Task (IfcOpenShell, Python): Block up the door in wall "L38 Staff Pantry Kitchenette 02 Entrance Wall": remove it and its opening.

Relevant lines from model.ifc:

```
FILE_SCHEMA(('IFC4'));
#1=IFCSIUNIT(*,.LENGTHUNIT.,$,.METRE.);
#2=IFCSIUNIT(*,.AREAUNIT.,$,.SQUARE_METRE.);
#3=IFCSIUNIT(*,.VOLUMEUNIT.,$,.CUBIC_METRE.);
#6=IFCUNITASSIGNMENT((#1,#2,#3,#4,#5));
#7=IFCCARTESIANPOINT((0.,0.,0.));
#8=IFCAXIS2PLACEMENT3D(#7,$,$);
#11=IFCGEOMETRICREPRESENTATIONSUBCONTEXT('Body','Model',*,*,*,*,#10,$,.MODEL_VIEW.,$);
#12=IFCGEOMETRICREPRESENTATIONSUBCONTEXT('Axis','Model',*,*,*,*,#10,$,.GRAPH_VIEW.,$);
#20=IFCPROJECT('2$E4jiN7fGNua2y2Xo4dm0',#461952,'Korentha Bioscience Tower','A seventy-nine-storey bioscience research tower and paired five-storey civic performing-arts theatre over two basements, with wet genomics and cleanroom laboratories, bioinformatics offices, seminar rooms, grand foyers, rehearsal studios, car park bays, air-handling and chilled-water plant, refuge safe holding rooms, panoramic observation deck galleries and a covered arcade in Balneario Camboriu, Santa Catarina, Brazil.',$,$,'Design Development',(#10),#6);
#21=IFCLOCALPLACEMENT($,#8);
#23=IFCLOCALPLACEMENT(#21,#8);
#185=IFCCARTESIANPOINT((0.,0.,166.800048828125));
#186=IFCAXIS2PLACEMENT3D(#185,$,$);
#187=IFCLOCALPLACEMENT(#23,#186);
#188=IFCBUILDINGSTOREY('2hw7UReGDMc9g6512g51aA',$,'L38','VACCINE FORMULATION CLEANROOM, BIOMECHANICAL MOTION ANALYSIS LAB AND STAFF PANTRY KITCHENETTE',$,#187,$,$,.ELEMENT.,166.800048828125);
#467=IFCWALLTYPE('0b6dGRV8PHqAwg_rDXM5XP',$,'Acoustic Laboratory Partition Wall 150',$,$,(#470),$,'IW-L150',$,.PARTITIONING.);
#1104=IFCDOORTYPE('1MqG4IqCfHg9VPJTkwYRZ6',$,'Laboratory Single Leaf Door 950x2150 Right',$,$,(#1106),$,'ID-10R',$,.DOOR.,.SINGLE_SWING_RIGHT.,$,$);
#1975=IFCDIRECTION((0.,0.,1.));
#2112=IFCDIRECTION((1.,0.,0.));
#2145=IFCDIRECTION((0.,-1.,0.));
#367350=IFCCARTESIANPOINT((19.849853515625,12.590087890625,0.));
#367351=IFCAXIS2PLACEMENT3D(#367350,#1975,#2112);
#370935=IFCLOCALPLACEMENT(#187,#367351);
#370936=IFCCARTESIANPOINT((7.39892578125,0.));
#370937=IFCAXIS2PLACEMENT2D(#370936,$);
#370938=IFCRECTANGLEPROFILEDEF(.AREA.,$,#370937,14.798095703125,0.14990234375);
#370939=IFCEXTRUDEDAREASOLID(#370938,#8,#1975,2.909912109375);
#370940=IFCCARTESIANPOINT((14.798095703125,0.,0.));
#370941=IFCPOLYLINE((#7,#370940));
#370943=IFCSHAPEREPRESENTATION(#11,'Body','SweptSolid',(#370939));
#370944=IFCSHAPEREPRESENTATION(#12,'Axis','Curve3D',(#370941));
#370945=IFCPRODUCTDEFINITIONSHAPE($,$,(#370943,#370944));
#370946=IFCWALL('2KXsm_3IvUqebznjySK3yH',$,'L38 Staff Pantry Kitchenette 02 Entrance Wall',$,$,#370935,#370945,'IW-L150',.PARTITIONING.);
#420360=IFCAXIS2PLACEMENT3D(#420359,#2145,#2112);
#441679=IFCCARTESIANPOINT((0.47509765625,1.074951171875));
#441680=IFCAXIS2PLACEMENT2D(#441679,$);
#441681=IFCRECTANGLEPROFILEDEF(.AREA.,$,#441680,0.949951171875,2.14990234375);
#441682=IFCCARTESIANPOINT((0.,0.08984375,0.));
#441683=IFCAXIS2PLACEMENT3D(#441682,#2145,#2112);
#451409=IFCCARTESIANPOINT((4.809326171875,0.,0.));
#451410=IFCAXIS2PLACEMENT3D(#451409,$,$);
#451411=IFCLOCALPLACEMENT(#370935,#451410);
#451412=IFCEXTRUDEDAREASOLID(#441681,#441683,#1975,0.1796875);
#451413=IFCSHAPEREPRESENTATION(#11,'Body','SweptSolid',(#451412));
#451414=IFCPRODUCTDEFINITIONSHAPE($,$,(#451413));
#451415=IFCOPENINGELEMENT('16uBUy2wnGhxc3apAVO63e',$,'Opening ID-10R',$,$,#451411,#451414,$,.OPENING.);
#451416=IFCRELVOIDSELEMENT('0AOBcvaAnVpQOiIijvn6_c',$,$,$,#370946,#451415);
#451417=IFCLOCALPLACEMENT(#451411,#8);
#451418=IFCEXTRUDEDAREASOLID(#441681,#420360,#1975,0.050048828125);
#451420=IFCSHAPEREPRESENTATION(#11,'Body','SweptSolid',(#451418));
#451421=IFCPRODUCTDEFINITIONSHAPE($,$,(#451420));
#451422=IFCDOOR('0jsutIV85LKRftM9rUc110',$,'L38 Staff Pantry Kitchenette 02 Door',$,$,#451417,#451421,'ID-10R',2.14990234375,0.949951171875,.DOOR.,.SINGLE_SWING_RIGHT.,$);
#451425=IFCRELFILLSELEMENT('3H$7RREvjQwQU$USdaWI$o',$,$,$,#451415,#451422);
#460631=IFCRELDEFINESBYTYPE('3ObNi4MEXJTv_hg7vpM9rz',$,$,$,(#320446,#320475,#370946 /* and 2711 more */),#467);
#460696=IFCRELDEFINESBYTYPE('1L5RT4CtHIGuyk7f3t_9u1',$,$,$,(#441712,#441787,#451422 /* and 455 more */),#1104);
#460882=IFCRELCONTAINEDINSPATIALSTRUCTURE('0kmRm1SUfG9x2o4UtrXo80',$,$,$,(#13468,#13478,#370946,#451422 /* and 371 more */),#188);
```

```python
import ifcopenshell
import ifcopenshell.api.feature
import ifcopenshell.api.root
import ifcopenshell.geom
import ifcopenshell.util.shape

model = ifcopenshell.open("model.ifc")
settings = ifcopenshell.geom.settings()


def volume(element):
    """Net volume in cubic metres, openings subtracted."""
    shape = ifcopenshell.geom.create_shape(settings, element)
    return ifcopenshell.util.shape.get_volume(shape.geometry)


door = model.by_guid("0jsutIV85LKRftM9rUc110")
opening = door.FillsVoids[0].RelatingOpeningElement
wall = opening.VoidsElements[0].RelatingBuildingElement
before = volume(wall)

ifcopenshell.api.root.remove_product(model, product=door)
ifcopenshell.api.feature.remove_feature(model, feature=opening)

after = volume(wall)

print(f"wall volume {before:.3f} -> {after:.3f} m3")

model.write("model_rev.ifc")
```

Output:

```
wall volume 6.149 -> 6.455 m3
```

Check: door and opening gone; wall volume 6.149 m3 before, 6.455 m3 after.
